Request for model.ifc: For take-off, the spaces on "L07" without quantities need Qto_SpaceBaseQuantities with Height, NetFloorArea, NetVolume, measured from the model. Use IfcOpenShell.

First a look at what the model holds.

```python
import ifcopenshell
import ifcopenshell.util.element
import ifcopenshell.util.unit

model = ifcopenshell.open("model.ifc")
print(model.schema)
for unit_type in ("LENGTHUNIT", "AREAUNIT", "VOLUMEUNIT"):
    print(unit_type, ifcopenshell.util.unit.calculate_unit_scale(model, unit_type))
storey = next(s for s in model.by_type("IfcBuildingStorey") if s.Name == "L07")
spaces = [e for e in ifcopenshell.util.element.get_decomposition(storey) if e.is_a("IfcSpace")]
for e in sorted(spaces, key=lambda e: e.id()):
    print(e.id(), e.is_a(), e.Name, list(ifcopenshell.util.element.get_psets(e, qtos_only=True)), sep=" | ")
```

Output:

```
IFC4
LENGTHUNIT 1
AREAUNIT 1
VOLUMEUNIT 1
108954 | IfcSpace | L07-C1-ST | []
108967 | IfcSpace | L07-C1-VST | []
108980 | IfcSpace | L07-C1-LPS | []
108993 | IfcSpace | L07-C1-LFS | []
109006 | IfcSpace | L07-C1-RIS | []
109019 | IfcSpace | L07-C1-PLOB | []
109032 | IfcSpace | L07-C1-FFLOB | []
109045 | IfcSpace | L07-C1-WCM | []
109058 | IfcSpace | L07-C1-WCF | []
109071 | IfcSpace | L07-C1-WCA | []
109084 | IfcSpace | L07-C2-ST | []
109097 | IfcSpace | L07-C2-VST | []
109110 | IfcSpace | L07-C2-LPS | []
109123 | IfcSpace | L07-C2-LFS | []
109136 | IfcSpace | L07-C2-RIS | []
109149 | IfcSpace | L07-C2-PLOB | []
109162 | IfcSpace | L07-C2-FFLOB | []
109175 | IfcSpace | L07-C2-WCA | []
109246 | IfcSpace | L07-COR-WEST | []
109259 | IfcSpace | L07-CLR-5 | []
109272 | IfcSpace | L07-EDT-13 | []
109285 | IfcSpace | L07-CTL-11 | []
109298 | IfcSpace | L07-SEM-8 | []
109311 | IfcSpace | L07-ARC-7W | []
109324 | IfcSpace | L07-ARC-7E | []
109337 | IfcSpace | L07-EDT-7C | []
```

```python
import ifcopenshell
import ifcopenshell.api.pset
import ifcopenshell.geom
import ifcopenshell.util.element
import ifcopenshell.util.shape
import ifcopenshell.util.unit

model = ifcopenshell.open("model.ifc")
unit_scale = ifcopenshell.util.unit.calculate_unit_scale(model)
area_scale = ifcopenshell.util.unit.calculate_unit_scale(model, "AREAUNIT")
volume_scale = ifcopenshell.util.unit.calculate_unit_scale(model, "VOLUMEUNIT")
settings = ifcopenshell.geom.settings()

storey = next(s for s in model.by_type("IfcBuildingStorey") if s.Name == "L07")
spaces = [e for e in ifcopenshell.util.element.get_decomposition(storey) if e.is_a("IfcSpace")]

for e in sorted(spaces, key=lambda e: e.id()):
    if ifcopenshell.util.element.get_psets(e, qtos_only=True, should_inherit=False):
        continue
    # Geometry comes back in metres, in the element's own axes.
    shape = ifcopenshell.geom.create_shape(settings, e)
    values = {
        "Height": ifcopenshell.util.shape.get_z(shape.geometry) / unit_scale,
        "NetFloorArea": ifcopenshell.util.shape.get_footprint_area(shape.geometry) / area_scale,
        "NetVolume": ifcopenshell.util.shape.get_volume(shape.geometry) / volume_scale,
    }
    qto = ifcopenshell.api.pset.add_qto(model, product=e, name="Qto_SpaceBaseQuantities")
    ifcopenshell.api.pset.edit_qto(model, qto=qto, properties=values)
    print(e.id(), {k: round(v, 3) for k, v in values.items()})

model.write("model_v2.ifc")
```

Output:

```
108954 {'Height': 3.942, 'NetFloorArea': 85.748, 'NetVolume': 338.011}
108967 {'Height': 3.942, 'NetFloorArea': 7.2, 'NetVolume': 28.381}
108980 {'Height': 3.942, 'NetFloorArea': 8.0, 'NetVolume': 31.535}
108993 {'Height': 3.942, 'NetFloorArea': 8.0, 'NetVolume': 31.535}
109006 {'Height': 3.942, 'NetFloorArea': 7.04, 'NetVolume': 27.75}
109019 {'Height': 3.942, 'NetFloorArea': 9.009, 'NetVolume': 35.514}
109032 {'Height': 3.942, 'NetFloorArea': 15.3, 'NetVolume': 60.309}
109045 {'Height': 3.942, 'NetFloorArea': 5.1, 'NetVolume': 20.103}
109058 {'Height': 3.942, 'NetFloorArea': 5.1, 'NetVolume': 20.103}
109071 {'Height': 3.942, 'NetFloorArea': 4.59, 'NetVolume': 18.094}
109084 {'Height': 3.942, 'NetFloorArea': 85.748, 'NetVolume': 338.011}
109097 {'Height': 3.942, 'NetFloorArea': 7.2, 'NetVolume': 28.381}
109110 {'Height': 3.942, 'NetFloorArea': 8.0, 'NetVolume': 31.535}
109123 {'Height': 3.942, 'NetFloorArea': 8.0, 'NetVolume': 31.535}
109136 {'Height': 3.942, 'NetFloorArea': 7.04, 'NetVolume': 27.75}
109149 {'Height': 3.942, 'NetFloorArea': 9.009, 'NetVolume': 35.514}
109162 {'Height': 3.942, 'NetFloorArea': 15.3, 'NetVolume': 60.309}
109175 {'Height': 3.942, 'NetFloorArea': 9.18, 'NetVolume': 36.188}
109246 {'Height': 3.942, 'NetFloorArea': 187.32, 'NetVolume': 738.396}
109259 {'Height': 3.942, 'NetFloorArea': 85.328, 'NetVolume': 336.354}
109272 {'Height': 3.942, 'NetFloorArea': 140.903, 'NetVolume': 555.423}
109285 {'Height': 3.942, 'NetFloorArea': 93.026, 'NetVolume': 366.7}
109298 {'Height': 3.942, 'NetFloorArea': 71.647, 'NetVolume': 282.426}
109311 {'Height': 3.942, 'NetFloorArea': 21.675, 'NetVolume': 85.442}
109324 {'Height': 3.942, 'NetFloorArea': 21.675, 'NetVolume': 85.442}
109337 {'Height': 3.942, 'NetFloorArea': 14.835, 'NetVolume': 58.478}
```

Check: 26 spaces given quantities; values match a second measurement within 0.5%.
